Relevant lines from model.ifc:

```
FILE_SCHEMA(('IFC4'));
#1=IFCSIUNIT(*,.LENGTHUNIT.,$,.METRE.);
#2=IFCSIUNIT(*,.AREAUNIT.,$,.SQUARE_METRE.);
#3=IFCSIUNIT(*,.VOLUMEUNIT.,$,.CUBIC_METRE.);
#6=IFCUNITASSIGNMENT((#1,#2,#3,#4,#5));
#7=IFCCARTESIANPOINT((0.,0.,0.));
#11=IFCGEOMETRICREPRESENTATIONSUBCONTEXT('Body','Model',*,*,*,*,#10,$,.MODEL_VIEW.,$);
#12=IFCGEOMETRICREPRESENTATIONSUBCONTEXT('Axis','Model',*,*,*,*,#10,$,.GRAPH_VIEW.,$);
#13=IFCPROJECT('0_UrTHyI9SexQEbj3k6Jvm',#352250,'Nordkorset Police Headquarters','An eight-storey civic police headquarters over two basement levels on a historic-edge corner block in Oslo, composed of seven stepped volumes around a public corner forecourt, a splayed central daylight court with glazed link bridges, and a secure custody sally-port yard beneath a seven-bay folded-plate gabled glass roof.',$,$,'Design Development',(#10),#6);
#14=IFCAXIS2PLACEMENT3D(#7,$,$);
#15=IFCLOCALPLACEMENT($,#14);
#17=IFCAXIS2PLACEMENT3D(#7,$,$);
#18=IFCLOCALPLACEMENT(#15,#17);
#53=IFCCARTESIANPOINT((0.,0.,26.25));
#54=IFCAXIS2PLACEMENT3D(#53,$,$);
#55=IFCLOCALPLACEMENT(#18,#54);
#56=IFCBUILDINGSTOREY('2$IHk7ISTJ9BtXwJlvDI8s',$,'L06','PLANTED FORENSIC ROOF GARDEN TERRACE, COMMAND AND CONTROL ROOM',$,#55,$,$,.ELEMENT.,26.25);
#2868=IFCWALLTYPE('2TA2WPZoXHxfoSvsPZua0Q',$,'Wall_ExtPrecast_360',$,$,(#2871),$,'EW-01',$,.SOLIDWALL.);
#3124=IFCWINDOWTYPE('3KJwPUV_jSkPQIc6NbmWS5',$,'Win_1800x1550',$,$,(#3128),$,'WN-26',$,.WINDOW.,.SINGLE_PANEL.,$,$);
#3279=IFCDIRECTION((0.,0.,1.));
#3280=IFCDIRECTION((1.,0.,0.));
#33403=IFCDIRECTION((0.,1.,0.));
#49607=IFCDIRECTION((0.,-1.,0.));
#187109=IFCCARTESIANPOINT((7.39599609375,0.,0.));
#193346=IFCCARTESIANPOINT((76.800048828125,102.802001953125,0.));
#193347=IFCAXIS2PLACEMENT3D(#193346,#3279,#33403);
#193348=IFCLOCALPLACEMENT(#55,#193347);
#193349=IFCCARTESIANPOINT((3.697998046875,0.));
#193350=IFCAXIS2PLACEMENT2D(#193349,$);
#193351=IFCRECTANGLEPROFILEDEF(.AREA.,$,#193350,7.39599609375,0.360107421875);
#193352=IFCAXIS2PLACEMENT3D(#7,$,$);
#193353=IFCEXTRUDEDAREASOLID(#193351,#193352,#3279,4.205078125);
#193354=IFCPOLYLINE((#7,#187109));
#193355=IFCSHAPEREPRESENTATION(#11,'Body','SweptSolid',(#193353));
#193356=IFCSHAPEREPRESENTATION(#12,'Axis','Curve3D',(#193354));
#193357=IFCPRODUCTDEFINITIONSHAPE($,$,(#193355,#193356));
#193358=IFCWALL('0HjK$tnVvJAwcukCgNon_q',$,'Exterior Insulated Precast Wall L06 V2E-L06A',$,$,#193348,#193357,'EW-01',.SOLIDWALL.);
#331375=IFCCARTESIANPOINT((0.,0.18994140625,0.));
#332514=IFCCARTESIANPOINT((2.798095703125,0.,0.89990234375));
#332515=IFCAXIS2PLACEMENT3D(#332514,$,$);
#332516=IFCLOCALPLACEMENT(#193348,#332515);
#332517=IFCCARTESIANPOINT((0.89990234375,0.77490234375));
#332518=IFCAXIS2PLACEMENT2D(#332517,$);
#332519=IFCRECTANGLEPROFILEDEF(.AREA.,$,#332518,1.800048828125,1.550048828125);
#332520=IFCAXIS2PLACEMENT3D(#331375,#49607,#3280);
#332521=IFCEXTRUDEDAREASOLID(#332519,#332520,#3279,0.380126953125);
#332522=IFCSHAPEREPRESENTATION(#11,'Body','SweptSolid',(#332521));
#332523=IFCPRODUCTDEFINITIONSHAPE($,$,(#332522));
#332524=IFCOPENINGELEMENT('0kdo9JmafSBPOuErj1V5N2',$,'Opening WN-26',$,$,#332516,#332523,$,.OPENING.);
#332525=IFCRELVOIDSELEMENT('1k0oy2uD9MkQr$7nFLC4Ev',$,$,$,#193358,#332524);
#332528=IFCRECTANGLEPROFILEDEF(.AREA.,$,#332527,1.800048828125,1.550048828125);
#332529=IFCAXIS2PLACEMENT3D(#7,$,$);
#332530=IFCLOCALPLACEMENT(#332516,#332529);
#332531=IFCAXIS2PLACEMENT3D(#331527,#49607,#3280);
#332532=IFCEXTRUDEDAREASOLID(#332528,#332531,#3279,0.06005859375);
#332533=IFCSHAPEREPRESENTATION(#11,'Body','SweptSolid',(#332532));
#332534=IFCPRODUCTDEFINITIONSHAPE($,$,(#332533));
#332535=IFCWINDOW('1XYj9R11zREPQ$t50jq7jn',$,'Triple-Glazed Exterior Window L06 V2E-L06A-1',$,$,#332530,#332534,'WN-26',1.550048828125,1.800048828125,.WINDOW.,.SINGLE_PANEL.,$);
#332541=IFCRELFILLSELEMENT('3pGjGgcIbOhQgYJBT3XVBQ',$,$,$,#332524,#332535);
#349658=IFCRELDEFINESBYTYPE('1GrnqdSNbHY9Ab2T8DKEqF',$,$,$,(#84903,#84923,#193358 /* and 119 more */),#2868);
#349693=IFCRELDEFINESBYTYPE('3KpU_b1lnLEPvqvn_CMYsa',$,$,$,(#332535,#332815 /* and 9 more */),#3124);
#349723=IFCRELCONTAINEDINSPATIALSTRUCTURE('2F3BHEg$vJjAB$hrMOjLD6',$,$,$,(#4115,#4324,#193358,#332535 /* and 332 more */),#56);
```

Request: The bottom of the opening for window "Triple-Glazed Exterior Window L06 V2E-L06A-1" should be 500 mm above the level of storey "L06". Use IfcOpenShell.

```python
import numpy as np
import ifcopenshell
import ifcopenshell.api.geometry
import ifcopenshell.geom
import ifcopenshell.util.element
import ifcopenshell.util.placement
import ifcopenshell.util.shape
import ifcopenshell.util.unit

model = ifcopenshell.open("model.ifc")
unit_scale = ifcopenshell.util.unit.calculate_unit_scale(model)

window = model.by_guid("1XYj9R11zREPQ$t50jq7jn")
opening = window.FillsVoids[0].RelatingOpeningElement
storey = ifcopenshell.util.element.get_container(window, ifc_class="IfcBuildingStorey")
level = ifcopenshell.util.placement.get_local_placement(storey.ObjectPlacement)[2, 3]

# The opening's origin need not be at the sill, so measure its lowest point.
shape = ifcopenshell.geom.create_shape(ifcopenshell.geom.settings(), opening)
bottom = ifcopenshell.util.shape.get_shape_bottom_elevation(shape, shape.geometry) / unit_scale
dz = level + 0.5 / unit_scale - bottom

shift = np.array([0.0, 0.0, dz])
# The window is placed relative to its opening, so it follows when the opening moves.
matrix = ifcopenshell.util.placement.get_local_placement(opening.ObjectPlacement)
matrix[:3, 3] += shift
ifcopenshell.api.geometry.edit_object_placement(
    model, product=opening, matrix=matrix, is_si=False, should_transform_children=True
)

print(f"moved by {dz * unit_scale:+.3f} m")

model.write("model_rev.ifc")
```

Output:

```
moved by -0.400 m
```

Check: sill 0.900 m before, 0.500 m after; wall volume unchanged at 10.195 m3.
